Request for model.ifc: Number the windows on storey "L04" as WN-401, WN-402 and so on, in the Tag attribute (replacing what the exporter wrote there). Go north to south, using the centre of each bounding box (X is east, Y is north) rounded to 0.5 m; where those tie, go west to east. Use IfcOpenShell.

First a look at what the model holds.

```python
import ifcopenshell
import ifcopenshell.util.element
import ifcopenshell.util.placement

model = ifcopenshell.open("model.ifc")
print(model.schema)
storey = next(s for s in model.by_type("IfcBuildingStorey") if s.Name == "L04")
windows = [e for e in ifcopenshell.util.element.get_decomposition(storey) if e.is_a("IfcWindow")]
for e in sorted(windows, key=lambda e: e.id()):
    origin = ifcopenshell.util.placement.get_local_placement(e.ObjectPlacement)[:3, 3]
    print(e.id(), e.Tag, e.Name, origin.round(2) + 0.0, sep=" | ")
```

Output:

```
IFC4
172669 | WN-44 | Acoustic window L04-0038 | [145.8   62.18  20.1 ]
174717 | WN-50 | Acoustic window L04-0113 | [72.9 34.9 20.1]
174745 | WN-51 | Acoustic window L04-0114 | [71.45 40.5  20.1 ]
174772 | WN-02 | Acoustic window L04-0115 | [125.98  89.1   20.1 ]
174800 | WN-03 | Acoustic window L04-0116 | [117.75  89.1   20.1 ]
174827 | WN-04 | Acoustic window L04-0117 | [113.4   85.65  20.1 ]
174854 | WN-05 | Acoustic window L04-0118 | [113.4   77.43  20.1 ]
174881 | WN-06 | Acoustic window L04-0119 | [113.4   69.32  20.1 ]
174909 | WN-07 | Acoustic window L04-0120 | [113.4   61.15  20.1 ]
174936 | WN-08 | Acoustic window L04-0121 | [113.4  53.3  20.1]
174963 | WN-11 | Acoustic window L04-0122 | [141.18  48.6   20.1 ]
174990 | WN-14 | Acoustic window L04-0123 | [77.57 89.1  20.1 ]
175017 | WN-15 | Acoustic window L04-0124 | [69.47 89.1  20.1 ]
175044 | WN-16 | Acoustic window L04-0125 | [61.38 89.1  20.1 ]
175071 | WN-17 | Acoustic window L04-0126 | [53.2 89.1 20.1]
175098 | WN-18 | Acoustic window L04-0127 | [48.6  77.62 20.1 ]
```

```python
import ifcopenshell
import ifcopenshell.geom
import ifcopenshell.util.element
import ifcopenshell.util.shape

model = ifcopenshell.open("model.ifc")
settings = ifcopenshell.geom.settings()
settings.set("use-world-coords", True)


def centre(element):
    shape = ifcopenshell.geom.create_shape(settings, element)
    return ifcopenshell.util.shape.get_bbox_centroid(shape.geometry)


storey = next(s for s in model.by_type("IfcBuildingStorey") if s.Name == "L04")
windows = [e for e in ifcopenshell.util.element.get_decomposition(storey) if e.is_a("IfcWindow")]

# Insertion points can sit at a corner or the storey origin, so sort by the geometry (in metres).
centres = {e: centre(e) for e in windows}
windows.sort(key=lambda e: (-round(centres[e][1] / 0.5), centres[e][0]))

for i, e in enumerate(windows, start=1):
    number = f"WN-4{i:02d}"
    e.Tag = number
    print(e.id(), number)

model.write("model-out.ifc")
```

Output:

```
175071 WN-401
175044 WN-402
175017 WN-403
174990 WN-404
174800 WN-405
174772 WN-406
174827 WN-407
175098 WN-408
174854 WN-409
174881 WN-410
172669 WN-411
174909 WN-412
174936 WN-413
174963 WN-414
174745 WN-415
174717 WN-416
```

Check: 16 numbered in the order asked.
